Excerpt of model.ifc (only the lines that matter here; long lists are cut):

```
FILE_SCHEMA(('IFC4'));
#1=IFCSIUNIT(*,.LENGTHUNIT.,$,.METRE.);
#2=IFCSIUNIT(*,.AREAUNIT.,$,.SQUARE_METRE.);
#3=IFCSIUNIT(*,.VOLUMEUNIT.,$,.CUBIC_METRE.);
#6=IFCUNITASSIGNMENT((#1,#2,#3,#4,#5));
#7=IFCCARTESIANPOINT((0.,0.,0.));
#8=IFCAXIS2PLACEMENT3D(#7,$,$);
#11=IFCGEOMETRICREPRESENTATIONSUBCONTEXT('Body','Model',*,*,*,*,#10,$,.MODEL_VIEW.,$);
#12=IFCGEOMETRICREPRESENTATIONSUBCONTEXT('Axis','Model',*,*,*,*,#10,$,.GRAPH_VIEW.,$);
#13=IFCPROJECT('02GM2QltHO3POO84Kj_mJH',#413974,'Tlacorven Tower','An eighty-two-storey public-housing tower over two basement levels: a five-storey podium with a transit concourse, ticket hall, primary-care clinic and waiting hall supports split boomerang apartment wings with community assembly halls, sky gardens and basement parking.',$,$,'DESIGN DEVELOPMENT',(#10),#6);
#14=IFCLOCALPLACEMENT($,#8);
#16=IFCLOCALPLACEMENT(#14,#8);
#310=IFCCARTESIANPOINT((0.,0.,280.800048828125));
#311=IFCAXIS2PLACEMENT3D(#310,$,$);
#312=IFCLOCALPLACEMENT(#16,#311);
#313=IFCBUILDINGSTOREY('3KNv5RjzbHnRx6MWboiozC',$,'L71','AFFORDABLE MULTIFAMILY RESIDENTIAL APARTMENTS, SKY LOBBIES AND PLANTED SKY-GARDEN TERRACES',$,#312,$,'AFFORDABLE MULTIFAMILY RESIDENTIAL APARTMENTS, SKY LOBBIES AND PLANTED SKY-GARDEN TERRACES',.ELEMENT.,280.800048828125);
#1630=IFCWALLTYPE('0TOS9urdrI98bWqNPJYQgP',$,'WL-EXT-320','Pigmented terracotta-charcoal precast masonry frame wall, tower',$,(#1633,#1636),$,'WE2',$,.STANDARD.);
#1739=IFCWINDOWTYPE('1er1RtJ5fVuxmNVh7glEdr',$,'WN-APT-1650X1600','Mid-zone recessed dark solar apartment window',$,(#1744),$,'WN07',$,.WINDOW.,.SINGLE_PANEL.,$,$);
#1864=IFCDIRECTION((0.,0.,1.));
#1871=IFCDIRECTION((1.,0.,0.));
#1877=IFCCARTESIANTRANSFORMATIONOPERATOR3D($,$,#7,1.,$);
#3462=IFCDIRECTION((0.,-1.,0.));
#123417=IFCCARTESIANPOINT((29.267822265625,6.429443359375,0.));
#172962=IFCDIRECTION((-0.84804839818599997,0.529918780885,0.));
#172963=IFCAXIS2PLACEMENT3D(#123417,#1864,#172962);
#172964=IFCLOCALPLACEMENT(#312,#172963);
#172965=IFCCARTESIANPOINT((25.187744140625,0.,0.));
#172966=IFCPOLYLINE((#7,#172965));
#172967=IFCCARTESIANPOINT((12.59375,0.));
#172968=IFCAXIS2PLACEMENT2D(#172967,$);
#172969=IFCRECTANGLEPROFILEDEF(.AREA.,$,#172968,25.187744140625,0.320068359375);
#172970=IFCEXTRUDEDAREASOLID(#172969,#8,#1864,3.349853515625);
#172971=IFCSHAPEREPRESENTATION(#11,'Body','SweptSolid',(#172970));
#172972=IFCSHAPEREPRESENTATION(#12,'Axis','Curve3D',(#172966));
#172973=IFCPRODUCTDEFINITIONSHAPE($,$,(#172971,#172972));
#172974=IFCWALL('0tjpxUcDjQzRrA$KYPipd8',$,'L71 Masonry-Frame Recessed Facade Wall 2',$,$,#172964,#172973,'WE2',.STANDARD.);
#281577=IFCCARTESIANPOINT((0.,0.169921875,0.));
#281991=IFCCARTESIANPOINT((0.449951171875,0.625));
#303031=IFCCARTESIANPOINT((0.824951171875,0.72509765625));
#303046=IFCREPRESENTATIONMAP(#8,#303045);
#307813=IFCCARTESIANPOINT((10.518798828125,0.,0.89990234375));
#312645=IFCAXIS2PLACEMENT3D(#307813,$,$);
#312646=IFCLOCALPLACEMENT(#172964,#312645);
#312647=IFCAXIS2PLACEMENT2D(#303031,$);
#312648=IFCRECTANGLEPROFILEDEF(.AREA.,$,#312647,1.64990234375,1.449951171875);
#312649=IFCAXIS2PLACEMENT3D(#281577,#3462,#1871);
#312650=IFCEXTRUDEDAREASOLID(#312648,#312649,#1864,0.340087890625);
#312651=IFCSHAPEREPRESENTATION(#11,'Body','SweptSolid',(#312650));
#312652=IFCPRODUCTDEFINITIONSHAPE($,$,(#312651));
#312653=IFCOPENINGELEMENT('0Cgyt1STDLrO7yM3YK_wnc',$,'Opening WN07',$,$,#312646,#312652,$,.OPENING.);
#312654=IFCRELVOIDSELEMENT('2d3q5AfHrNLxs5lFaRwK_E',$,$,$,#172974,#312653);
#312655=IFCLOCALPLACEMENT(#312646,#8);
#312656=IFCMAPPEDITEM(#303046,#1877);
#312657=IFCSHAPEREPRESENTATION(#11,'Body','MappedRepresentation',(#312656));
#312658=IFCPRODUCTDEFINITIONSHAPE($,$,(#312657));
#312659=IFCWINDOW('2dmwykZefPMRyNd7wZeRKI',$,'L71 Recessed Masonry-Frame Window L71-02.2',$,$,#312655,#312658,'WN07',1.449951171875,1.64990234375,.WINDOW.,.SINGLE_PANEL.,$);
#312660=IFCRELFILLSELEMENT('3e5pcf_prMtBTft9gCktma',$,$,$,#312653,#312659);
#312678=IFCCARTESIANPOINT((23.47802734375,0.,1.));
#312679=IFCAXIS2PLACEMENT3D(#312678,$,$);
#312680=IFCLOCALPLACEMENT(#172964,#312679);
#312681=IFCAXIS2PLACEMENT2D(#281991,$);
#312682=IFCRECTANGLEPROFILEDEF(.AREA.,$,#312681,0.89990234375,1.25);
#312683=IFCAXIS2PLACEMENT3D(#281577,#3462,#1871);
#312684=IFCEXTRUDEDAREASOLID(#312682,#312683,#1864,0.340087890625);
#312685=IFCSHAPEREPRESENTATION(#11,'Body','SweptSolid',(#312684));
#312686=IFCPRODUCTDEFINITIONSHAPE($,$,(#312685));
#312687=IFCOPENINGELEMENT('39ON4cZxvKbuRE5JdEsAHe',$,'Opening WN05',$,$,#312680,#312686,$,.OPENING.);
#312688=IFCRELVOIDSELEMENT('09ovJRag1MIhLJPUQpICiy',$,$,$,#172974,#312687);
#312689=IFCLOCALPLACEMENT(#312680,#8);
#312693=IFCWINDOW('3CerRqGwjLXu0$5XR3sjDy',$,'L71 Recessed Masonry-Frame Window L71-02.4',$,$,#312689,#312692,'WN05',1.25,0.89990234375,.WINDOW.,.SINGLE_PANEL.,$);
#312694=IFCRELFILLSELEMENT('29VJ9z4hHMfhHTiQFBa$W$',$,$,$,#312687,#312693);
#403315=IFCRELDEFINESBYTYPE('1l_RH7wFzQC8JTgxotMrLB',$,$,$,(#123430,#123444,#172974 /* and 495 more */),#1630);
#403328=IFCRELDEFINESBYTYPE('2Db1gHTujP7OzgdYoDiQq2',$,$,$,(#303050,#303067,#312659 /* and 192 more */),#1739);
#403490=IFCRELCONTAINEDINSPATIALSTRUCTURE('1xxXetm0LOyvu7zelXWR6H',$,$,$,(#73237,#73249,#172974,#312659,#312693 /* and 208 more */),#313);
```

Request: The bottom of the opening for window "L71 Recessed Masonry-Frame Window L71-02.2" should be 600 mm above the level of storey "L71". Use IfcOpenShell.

```python
import numpy as np
import ifcopenshell
import ifcopenshell.api.geometry
import ifcopenshell.geom
import ifcopenshell.util.element
import ifcopenshell.util.placement
import ifcopenshell.util.shape
import ifcopenshell.util.unit

model = ifcopenshell.open("model.ifc")
unit_scale = ifcopenshell.util.unit.calculate_unit_scale(model)

window = model.by_guid("2dmwykZefPMRyNd7wZeRKI")
opening = window.FillsVoids[0].RelatingOpeningElement
storey = ifcopenshell.util.element.get_container(window, ifc_class="IfcBuildingStorey")
level = ifcopenshell.util.placement.get_local_placement(storey.ObjectPlacement)[2, 3]

# The opening's origin need not be at the sill, so measure its lowest point.
shape = ifcopenshell.geom.create_shape(ifcopenshell.geom.settings(), opening)
bottom = ifcopenshell.util.shape.get_shape_bottom_elevation(shape, shape.geometry) / unit_scale
dz = level + 0.6 / unit_scale - bottom

shift = np.array([0.0, 0.0, dz])
# The window is placed relative to its opening, so it follows when the opening moves.
matrix = ifcopenshell.util.placement.get_local_placement(opening.ObjectPlacement)
matrix[:3, 3] += shift
ifcopenshell.api.geometry.edit_object_placement(
    model, product=opening, matrix=matrix, is_si=False, should_transform_children=True
)

print(f"moved by {dz * unit_scale:+.3f} m")

model.write("model-out.ifc")
```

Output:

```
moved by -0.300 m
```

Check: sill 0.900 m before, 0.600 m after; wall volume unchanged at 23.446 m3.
